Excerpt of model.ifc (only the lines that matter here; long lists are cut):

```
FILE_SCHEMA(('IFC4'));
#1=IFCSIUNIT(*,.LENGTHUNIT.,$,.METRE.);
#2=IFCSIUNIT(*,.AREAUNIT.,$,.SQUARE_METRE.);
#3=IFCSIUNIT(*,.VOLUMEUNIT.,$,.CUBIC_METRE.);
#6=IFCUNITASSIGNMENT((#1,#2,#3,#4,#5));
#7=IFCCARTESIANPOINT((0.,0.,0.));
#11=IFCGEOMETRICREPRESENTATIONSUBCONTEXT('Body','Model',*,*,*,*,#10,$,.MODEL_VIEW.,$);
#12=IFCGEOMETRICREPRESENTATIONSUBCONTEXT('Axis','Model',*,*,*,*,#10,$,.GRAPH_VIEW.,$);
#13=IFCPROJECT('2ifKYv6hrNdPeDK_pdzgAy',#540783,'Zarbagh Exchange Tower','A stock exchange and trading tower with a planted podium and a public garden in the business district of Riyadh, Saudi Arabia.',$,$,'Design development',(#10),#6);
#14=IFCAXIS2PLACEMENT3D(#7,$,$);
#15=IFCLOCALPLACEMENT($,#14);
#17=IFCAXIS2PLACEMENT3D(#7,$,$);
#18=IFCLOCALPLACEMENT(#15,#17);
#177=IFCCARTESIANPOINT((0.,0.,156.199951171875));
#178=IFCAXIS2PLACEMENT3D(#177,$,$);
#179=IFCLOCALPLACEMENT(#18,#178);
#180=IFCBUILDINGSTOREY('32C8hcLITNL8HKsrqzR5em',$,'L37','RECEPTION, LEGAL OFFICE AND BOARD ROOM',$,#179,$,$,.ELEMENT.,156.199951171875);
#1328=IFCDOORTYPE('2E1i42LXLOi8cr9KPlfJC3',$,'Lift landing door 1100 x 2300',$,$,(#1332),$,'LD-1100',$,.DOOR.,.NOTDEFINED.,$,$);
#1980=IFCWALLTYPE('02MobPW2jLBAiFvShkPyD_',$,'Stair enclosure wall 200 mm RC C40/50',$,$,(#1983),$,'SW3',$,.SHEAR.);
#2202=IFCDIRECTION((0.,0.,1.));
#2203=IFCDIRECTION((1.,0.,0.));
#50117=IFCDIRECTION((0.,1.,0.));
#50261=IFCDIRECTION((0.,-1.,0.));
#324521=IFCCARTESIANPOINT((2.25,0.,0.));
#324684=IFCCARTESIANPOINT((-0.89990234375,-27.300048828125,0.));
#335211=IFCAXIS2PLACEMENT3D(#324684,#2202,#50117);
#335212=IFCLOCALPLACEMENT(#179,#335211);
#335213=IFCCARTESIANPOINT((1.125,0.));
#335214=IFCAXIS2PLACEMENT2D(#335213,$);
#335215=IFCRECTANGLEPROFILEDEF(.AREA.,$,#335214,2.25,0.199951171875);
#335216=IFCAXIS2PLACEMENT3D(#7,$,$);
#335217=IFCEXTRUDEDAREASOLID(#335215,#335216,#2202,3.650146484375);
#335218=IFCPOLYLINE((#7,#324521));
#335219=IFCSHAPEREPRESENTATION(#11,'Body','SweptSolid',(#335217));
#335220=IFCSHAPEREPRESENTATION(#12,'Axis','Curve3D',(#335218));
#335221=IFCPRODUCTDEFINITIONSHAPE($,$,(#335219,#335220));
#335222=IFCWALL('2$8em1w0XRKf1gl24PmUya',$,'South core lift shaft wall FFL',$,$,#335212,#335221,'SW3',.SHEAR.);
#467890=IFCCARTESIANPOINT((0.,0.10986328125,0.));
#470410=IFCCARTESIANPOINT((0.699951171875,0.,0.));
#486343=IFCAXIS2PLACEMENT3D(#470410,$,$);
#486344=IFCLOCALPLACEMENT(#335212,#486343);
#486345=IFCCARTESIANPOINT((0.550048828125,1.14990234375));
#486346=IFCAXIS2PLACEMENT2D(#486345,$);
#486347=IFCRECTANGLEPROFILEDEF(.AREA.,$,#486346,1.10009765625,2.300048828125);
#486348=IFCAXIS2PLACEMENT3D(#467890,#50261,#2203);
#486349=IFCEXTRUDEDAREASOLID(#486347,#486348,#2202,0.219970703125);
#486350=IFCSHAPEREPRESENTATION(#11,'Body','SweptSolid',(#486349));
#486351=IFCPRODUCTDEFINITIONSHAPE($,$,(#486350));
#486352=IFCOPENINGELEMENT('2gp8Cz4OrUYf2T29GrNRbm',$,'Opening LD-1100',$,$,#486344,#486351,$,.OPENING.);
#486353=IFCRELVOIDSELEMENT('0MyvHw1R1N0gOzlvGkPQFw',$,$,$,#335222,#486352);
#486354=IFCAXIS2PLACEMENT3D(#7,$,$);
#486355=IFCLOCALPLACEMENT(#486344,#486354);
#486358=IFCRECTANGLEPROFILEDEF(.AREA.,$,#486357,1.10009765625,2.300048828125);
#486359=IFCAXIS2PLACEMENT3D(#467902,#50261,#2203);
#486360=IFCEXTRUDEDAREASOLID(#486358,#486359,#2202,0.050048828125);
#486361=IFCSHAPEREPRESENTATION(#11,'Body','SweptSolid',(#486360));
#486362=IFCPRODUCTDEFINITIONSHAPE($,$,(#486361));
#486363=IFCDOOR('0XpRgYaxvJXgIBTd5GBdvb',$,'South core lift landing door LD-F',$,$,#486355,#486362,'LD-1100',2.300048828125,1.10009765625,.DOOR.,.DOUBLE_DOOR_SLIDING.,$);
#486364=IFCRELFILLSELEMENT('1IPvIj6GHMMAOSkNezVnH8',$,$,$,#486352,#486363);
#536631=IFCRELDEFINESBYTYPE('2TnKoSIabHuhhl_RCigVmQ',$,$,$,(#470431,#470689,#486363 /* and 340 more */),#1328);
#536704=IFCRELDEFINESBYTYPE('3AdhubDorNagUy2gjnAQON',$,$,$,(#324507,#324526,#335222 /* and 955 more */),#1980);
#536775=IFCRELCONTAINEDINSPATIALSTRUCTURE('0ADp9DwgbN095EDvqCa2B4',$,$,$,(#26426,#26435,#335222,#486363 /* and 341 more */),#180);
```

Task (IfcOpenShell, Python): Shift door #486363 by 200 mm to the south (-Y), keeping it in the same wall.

```python
import ifcopenshell
import ifcopenshell.api.geometry
import ifcopenshell.util.placement
import ifcopenshell.util.unit

model = ifcopenshell.open("model.ifc")
unit_scale = ifcopenshell.util.unit.calculate_unit_scale(model)

door = model.by_id(486363)
opening = door.FillsVoids[0].RelatingOpeningElement
wall = opening.VoidsElements[0].RelatingBuildingElement

wall_matrix = ifcopenshell.util.placement.get_local_placement(wall.ObjectPlacement)
shift = wall_matrix[:3, 0] * -0.2 / unit_scale
before = ifcopenshell.util.placement.get_local_placement(door.ObjectPlacement)[:3, 3].copy()

# The door is placed relative to its opening, so it follows when the opening moves.
matrix = ifcopenshell.util.placement.get_local_placement(opening.ObjectPlacement)
matrix[:3, 3] += shift
ifcopenshell.api.geometry.edit_object_placement(
    model, product=opening, matrix=matrix, is_si=False, should_transform_children=True
)

after = ifcopenshell.util.placement.get_local_placement(door.ObjectPlacement)[:3, 3]
print("door moved by", (after - before).round(3) + 0.0)

model.write("model_v2.ifc")
```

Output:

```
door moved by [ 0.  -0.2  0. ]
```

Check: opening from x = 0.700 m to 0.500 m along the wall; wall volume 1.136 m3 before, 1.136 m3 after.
